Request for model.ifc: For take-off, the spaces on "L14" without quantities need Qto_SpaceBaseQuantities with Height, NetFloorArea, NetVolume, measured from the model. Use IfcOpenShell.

First a look at what the model holds.

```python
import ifcopenshell
import ifcopenshell.util.element
import ifcopenshell.util.unit

model = ifcopenshell.open("model.ifc")
print(model.schema)
for unit_type in ("LENGTHUNIT", "AREAUNIT", "VOLUMEUNIT"):
    print(unit_type, ifcopenshell.util.unit.calculate_unit_scale(model, unit_type))
storey = next(s for s in model.by_type("IfcBuildingStorey") if s.Name == "L14")
spaces = [e for e in ifcopenshell.util.element.get_decomposition(storey) if e.is_a("IfcSpace")]
for e in sorted(spaces, key=lambda e: e.id()):
    print(e.id(), e.is_a(), e.Name, list(ifcopenshell.util.element.get_psets(e, qtos_only=True)), sep=" | ")
```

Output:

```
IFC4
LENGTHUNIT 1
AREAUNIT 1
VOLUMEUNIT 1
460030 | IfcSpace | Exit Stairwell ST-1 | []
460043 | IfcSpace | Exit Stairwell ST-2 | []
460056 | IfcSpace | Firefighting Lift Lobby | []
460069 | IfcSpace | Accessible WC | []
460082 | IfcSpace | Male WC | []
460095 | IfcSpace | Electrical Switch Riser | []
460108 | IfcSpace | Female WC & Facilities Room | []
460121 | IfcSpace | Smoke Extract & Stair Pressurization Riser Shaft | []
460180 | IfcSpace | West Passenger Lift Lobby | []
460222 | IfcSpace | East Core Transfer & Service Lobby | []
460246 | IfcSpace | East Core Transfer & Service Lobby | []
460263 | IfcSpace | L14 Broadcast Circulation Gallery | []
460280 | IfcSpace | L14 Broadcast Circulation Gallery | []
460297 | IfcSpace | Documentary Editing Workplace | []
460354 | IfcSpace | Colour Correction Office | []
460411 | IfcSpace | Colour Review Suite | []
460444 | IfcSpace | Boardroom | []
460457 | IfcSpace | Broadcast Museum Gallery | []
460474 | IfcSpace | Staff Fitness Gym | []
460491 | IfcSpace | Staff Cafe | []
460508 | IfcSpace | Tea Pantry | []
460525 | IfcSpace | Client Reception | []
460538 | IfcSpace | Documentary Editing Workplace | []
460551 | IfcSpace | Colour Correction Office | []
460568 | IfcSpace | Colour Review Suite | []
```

```python
import ifcopenshell
import ifcopenshell.api.pset
import ifcopenshell.geom
import ifcopenshell.util.element
import ifcopenshell.util.shape
import ifcopenshell.util.unit

model = ifcopenshell.open("model.ifc")
unit_scale = ifcopenshell.util.unit.calculate_unit_scale(model)
area_scale = ifcopenshell.util.unit.calculate_unit_scale(model, "AREAUNIT")
volume_scale = ifcopenshell.util.unit.calculate_unit_scale(model, "VOLUMEUNIT")
settings = ifcopenshell.geom.settings()

storey = next(s for s in model.by_type("IfcBuildingStorey") if s.Name == "L14")
spaces = [e for e in ifcopenshell.util.element.get_decomposition(storey) if e.is_a("IfcSpace")]

for e in sorted(spaces, key=lambda e: e.id()):
    if ifcopenshell.util.element.get_psets(e, qtos_only=True, should_inherit=False):
        continue
    # Geometry comes back in metres, in the element's own axes.
    shape = ifcopenshell.geom.create_shape(settings, e)
    values = {
        "Height": ifcopenshell.util.shape.get_z(shape.geometry) / unit_scale,
        "NetFloorArea": ifcopenshell.util.shape.get_footprint_area(shape.geometry) / area_scale,
        "NetVolume": ifcopenshell.util.shape.get_volume(shape.geometry) / volume_scale,
    }
    qto = ifcopenshell.api.pset.add_qto(model, product=e, name="Qto_SpaceBaseQuantities")
    ifcopenshell.api.pset.edit_qto(model, qto=qto, properties=values)
    print(e.id(), {k: round(v, 3) for k, v in values.items()})

model.write("model_v2.ifc")
```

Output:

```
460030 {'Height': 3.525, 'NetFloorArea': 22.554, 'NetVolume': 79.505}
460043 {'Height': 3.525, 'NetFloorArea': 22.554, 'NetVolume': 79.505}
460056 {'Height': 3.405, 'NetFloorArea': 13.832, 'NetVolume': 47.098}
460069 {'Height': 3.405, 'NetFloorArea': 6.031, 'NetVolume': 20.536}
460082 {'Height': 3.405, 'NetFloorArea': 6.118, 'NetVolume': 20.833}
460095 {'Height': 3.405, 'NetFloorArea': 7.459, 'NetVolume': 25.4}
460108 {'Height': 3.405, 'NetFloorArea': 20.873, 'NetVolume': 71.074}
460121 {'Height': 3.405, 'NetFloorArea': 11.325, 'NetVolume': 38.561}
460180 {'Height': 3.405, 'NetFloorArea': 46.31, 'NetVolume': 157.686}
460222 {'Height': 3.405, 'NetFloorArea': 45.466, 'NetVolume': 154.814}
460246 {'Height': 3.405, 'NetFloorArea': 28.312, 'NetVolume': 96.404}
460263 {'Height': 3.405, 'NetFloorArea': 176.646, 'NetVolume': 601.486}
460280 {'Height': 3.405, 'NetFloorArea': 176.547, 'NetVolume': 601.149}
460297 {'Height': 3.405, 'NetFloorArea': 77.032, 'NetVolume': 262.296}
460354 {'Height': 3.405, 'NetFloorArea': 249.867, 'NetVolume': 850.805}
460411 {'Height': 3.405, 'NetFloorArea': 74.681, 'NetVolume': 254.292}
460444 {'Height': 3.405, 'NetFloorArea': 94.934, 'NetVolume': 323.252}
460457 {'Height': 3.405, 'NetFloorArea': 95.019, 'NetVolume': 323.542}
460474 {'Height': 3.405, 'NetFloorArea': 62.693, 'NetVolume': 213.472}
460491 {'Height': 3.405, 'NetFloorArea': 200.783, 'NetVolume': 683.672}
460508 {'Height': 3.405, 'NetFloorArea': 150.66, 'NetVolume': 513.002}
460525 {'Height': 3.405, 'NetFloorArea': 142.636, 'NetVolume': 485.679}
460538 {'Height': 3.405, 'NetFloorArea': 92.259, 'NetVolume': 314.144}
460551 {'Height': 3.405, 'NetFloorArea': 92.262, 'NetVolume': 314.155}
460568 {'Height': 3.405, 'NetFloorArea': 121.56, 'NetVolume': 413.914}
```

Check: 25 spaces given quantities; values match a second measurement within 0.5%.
